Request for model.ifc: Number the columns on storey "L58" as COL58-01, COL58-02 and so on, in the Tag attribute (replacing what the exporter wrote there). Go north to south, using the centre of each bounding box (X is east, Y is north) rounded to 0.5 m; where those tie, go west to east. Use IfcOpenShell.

First a look at what the model holds.

```python
import ifcopenshell
import ifcopenshell.util.element
import ifcopenshell.util.placement

model = ifcopenshell.open("model.ifc")
print(model.schema)
storey = next(s for s in model.by_type("IfcBuildingStorey") if s.Name == "L58")
columns = [e for e in ifcopenshell.util.element.get_decomposition(storey) if e.is_a("IfcColumn")]
for e in sorted(columns, key=lambda e: e.id()):
    origin = ifcopenshell.util.placement.get_local_placement(e.ObjectPlacement)[:3, 3]
    print(e.id(), e.Tag, e.Name, origin.round(2) + 0.0, sep=" | ")
```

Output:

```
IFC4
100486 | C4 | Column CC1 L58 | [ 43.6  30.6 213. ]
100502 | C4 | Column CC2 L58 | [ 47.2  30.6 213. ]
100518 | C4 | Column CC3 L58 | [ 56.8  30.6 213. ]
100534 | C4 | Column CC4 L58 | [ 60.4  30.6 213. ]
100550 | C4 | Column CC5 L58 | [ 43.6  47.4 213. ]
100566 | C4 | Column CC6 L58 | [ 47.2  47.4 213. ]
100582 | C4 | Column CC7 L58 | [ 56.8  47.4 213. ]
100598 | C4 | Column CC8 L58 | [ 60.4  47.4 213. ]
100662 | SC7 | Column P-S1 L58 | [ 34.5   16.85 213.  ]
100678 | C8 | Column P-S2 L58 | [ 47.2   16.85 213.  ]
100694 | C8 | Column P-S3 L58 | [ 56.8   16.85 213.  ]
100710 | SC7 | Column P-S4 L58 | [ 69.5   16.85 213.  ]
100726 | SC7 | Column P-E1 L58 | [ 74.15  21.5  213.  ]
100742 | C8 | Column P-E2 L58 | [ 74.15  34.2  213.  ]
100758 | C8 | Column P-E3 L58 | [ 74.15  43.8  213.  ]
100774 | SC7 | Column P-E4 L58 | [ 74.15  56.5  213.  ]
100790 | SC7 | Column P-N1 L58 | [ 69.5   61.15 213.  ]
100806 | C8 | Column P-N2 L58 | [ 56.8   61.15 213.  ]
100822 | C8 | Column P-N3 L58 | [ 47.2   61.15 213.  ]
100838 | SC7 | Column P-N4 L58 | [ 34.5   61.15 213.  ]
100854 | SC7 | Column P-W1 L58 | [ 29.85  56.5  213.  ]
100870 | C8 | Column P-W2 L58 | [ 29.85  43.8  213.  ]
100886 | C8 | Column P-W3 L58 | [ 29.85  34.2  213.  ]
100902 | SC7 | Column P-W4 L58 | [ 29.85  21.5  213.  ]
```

```python
import ifcopenshell
import ifcopenshell.geom
import ifcopenshell.util.element
import ifcopenshell.util.shape

model = ifcopenshell.open("model.ifc")
settings = ifcopenshell.geom.settings()
settings.set("use-world-coords", True)


def centre(element):
    shape = ifcopenshell.geom.create_shape(settings, element)
    return ifcopenshell.util.shape.get_bbox_centroid(shape.geometry)


storey = next(s for s in model.by_type("IfcBuildingStorey") if s.Name == "L58")
columns = [e for e in ifcopenshell.util.element.get_decomposition(storey) if e.is_a("IfcColumn")]

# Insertion points can sit at a corner or the storey origin, so sort by the geometry (in metres).
centres = {e: centre(e) for e in columns}
columns.sort(key=lambda e: (-round(centres[e][1] / 0.5), centres[e][0]))

for i, e in enumerate(columns, start=1):
    number = f"COL58-{i:02d}"
    e.Tag = number
    print(e.id(), number)

model.write("model_edited.ifc")
```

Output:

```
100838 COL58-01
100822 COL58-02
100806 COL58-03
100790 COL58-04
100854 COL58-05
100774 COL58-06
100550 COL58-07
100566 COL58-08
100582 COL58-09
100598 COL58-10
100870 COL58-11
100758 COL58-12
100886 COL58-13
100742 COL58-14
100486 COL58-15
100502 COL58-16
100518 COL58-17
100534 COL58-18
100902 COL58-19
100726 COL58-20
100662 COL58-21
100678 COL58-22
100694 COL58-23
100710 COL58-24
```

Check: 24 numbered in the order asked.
